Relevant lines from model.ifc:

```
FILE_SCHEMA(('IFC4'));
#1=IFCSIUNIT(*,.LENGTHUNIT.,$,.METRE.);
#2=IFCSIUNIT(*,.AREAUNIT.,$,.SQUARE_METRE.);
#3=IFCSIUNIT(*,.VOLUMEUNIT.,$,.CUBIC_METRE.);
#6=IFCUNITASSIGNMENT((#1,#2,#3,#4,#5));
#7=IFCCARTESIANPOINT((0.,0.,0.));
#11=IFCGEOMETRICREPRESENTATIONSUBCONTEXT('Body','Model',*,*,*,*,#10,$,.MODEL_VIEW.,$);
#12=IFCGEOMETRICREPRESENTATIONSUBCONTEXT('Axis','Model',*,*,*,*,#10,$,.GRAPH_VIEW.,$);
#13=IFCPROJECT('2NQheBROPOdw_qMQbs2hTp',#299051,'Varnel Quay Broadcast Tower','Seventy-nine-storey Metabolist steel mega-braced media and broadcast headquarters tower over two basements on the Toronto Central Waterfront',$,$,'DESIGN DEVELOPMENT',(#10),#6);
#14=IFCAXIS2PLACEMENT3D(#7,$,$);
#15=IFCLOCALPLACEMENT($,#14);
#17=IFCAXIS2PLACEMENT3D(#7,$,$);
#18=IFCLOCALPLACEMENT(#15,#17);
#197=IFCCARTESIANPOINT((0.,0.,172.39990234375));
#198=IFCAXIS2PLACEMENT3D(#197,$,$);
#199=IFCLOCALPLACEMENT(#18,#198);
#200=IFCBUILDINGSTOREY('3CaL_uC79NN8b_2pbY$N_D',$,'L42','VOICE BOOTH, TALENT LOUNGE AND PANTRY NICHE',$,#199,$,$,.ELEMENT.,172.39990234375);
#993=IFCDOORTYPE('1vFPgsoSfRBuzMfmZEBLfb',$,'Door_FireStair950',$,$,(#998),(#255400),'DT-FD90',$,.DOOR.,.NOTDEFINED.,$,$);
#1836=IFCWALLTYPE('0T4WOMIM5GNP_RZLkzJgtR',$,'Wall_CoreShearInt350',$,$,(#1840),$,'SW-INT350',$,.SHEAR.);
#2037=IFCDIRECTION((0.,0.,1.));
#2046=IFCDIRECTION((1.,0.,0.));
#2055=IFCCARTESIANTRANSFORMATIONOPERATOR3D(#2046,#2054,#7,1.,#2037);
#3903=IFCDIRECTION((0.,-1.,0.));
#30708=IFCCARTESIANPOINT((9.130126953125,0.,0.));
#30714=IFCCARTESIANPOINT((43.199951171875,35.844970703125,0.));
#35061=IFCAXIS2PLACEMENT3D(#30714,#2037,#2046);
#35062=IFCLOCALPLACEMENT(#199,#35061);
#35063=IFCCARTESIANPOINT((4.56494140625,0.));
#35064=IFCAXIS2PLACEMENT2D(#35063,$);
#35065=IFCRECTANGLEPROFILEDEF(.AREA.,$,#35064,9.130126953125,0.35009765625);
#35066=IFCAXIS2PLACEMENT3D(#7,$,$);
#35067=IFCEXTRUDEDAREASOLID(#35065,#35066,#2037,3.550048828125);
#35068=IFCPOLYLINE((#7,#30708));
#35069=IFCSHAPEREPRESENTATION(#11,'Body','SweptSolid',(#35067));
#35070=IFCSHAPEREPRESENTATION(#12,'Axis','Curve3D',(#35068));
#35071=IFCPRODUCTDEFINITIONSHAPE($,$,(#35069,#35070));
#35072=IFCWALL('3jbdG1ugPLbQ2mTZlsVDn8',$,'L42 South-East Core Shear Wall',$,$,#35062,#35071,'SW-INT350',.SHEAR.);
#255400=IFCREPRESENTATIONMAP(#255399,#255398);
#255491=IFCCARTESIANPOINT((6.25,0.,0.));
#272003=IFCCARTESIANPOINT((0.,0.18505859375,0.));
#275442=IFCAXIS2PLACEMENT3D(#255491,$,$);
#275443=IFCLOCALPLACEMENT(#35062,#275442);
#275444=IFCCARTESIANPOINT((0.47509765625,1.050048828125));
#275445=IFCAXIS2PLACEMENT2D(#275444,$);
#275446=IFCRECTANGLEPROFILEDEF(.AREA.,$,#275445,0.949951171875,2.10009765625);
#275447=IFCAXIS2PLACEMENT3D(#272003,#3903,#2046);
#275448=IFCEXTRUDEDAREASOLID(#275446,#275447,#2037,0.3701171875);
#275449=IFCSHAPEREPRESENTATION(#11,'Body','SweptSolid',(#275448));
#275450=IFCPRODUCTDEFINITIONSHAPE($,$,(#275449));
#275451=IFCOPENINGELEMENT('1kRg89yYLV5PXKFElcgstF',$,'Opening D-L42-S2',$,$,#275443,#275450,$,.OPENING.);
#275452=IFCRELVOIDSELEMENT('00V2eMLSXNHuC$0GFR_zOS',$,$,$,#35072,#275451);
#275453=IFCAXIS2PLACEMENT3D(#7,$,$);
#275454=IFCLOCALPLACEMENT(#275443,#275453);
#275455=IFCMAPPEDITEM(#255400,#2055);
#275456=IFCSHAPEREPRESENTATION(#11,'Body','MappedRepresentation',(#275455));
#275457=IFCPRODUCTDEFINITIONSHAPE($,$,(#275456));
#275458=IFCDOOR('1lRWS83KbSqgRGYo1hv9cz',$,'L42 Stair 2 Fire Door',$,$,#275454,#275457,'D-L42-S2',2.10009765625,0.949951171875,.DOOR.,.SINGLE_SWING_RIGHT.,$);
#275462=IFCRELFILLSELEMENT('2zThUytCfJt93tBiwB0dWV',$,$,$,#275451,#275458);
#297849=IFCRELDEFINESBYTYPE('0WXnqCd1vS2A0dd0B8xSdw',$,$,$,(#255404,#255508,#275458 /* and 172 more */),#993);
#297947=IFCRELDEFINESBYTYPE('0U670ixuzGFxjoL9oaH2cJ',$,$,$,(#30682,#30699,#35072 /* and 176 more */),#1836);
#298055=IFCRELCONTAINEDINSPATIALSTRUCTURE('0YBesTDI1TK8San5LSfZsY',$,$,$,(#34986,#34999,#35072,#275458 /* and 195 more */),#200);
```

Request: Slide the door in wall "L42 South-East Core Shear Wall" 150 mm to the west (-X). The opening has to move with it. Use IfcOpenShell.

```python
import ifcopenshell
import ifcopenshell.api.geometry
import ifcopenshell.util.placement

model = ifcopenshell.open("model.ifc")

door = model.by_id(275458)
opening = door.FillsVoids[0].RelatingOpeningElement
wall = opening.VoidsElements[0].RelatingBuildingElement

wall_matrix = ifcopenshell.util.placement.get_local_placement(wall.ObjectPlacement)
shift = wall_matrix[:3, 0] * -0.15
before = ifcopenshell.util.placement.get_local_placement(door.ObjectPlacement)[:3, 3].copy()

# The door is placed relative to its opening, so it follows when the opening moves.
matrix = ifcopenshell.util.placement.get_local_placement(opening.ObjectPlacement)
matrix[:3, 3] += shift
ifcopenshell.api.geometry.edit_object_placement(
    model, product=opening, matrix=matrix, is_si=False, should_transform_children=True
)

after = ifcopenshell.util.placement.get_local_placement(door.ObjectPlacement)[:3, 3]
print("door moved by", (after - before).round(3) + 0.0)

model.write("model_updated.ifc")
```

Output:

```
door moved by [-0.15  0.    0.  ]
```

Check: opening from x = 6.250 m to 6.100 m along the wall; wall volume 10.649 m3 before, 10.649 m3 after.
